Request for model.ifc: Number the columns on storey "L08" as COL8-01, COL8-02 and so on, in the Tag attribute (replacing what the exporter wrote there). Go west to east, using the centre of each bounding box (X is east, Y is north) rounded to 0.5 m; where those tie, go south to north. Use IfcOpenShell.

First a look at what the model holds.

```python
import ifcopenshell
import ifcopenshell.util.element
import ifcopenshell.util.placement

model = ifcopenshell.open("model.ifc")
print(model.schema)
storey = next(s for s in model.by_type("IfcBuildingStorey") if s.Name == "L08")
columns = [e for e in ifcopenshell.util.element.get_decomposition(storey) if e.is_a("IfcColumn")]
for e in sorted(columns, key=lambda e: e.id()):
    origin = ifcopenshell.util.placement.get_local_placement(e.ObjectPlacement)[:3, 3]
    print(e.id(), e.Tag, e.Name, origin.round(2) + 0.0, sep=" | ")
```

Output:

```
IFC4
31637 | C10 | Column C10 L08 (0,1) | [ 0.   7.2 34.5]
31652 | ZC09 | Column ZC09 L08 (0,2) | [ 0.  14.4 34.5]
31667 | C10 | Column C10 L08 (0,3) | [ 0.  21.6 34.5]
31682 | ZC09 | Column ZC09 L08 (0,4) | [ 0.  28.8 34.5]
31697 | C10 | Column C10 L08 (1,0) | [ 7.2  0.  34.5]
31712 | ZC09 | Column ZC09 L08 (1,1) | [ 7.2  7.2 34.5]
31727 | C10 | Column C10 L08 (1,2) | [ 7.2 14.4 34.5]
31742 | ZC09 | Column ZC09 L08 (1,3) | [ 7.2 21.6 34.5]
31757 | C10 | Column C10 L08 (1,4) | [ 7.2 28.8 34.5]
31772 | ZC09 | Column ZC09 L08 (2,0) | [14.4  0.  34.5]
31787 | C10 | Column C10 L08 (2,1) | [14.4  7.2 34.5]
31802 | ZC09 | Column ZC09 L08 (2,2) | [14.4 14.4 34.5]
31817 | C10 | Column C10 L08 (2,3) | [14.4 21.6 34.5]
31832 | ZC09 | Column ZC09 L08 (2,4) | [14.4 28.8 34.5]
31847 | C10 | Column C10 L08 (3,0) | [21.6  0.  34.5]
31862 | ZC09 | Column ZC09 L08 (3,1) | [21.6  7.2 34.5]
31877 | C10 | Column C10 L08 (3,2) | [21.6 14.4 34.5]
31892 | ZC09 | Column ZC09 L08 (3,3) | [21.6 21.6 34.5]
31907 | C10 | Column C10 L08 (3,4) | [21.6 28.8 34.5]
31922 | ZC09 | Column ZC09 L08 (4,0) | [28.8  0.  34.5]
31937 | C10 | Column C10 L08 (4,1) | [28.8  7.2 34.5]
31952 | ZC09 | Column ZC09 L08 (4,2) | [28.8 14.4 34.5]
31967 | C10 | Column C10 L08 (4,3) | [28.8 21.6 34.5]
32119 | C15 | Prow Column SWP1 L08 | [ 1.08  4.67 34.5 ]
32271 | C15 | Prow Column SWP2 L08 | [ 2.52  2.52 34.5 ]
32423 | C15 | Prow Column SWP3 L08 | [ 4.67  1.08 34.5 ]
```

```python
import ifcopenshell
import ifcopenshell.geom
import ifcopenshell.util.element
import ifcopenshell.util.shape

model = ifcopenshell.open("model.ifc")
settings = ifcopenshell.geom.settings()
settings.set("use-world-coords", True)


def centre(element):
    shape = ifcopenshell.geom.create_shape(settings, element)
    return ifcopenshell.util.shape.get_bbox_centroid(shape.geometry)


storey = next(s for s in model.by_type("IfcBuildingStorey") if s.Name == "L08")
columns = [e for e in ifcopenshell.util.element.get_decomposition(storey) if e.is_a("IfcColumn")]

# Insertion points can sit at a corner or the storey origin, so sort by the geometry (in metres).
centres = {e: centre(e) for e in columns}
columns.sort(key=lambda e: (round(centres[e][0] / 0.5), centres[e][1]))

for i, e in enumerate(columns, start=1):
    number = f"COL8-{i:02d}"
    e.Tag = number
    print(e.id(), number)

model.write("model_rev.ifc")
```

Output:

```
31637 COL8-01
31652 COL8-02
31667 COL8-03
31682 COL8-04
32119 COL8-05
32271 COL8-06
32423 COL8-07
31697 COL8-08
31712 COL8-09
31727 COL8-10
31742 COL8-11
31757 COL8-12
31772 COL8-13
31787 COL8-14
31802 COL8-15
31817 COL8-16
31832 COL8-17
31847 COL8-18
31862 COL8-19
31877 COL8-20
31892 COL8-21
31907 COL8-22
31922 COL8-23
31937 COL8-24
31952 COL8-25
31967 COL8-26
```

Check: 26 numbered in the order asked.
